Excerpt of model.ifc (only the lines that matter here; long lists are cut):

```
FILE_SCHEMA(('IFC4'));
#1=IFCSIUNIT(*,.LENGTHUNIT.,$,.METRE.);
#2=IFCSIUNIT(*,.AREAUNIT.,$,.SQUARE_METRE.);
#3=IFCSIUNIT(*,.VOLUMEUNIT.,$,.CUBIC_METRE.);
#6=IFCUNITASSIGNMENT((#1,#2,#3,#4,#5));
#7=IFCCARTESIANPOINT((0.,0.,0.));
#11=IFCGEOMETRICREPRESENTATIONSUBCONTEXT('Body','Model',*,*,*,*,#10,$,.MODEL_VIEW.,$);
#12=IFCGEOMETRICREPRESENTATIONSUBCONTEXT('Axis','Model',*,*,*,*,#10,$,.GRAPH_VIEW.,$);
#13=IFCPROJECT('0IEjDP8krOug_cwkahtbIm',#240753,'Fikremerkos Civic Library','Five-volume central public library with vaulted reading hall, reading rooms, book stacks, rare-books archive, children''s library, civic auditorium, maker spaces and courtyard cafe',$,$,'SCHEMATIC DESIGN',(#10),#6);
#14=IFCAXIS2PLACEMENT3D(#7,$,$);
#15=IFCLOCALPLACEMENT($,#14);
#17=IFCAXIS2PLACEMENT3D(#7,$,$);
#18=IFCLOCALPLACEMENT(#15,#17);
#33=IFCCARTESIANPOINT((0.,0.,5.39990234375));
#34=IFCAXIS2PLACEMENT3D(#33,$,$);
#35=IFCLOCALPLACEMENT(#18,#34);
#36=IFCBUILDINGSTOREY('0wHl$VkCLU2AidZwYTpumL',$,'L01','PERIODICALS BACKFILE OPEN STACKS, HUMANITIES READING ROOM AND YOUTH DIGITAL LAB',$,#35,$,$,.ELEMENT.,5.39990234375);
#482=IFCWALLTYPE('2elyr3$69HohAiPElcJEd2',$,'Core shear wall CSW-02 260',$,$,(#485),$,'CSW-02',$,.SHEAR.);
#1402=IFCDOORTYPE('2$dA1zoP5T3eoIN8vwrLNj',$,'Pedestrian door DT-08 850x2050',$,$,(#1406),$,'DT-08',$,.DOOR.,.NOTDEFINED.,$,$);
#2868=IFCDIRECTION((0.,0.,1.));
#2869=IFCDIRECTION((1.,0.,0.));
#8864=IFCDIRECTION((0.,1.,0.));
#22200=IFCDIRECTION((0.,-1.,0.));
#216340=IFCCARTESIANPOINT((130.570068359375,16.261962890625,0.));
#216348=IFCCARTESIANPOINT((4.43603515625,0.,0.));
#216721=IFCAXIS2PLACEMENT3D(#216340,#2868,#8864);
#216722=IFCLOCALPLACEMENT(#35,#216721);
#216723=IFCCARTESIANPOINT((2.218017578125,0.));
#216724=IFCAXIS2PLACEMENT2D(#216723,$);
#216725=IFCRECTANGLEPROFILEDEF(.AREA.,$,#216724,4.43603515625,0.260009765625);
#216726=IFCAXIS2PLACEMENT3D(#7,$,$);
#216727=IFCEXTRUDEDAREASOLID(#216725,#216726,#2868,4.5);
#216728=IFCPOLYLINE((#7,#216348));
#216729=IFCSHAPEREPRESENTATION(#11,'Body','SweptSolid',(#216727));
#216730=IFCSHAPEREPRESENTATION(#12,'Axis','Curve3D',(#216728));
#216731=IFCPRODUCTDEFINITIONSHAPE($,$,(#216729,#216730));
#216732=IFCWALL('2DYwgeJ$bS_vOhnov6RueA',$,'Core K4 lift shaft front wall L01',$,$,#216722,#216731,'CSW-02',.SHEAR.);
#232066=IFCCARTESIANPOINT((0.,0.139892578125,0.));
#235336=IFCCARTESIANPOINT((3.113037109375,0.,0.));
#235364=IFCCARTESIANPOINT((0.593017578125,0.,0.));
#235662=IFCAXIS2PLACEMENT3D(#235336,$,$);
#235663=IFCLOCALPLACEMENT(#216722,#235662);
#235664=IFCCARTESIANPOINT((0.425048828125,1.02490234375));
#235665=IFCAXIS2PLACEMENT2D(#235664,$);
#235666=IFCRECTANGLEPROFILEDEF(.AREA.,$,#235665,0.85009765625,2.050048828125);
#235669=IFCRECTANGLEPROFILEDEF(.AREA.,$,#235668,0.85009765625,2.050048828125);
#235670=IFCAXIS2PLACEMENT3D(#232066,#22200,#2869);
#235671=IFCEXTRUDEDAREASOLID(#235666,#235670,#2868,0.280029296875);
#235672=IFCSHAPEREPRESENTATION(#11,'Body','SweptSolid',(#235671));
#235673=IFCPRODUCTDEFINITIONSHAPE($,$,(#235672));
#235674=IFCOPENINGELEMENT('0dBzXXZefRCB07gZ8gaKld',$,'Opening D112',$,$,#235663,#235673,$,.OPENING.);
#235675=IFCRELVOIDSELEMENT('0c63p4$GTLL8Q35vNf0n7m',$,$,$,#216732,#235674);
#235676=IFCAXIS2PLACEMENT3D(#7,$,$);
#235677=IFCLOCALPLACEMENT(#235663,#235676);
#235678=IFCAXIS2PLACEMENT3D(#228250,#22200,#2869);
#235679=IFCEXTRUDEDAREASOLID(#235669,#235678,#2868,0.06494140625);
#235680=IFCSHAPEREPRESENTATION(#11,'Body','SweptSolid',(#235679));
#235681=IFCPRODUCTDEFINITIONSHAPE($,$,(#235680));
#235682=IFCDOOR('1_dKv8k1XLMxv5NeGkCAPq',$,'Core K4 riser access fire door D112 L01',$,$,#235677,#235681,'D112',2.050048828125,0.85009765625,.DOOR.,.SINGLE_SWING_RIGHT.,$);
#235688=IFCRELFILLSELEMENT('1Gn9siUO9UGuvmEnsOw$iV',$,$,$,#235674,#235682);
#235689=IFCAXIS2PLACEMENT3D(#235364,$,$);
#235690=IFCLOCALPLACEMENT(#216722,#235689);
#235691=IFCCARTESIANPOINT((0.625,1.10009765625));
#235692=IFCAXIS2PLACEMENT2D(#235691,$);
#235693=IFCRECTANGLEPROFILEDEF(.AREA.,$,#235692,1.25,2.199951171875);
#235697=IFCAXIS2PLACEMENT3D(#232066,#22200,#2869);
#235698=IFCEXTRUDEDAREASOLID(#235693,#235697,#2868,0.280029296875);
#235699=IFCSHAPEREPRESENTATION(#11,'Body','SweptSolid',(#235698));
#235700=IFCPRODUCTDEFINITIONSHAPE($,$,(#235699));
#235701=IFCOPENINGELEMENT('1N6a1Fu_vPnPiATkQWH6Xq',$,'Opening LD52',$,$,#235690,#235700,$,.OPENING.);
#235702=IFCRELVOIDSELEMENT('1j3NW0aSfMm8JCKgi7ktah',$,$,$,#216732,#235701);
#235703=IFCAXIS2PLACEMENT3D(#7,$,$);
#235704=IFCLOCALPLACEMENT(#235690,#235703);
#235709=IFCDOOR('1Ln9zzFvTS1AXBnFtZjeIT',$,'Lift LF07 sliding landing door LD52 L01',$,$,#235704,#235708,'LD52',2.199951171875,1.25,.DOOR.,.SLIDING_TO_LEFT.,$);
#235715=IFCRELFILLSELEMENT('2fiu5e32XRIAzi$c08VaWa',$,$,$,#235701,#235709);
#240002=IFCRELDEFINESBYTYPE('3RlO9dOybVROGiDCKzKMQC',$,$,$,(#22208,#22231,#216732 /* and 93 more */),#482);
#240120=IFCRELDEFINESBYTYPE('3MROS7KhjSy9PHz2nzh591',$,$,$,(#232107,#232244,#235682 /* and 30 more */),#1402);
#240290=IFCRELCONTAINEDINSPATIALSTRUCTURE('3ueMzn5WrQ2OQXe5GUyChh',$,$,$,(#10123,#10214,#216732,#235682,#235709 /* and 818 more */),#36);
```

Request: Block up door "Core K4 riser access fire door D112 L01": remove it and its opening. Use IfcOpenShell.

```python
import ifcopenshell
import ifcopenshell.api.feature
import ifcopenshell.api.root
import ifcopenshell.geom
import ifcopenshell.util.shape

model = ifcopenshell.open("model.ifc")
settings = ifcopenshell.geom.settings()


def volume(element):
    """Net volume in cubic metres, openings subtracted."""
    shape = ifcopenshell.geom.create_shape(settings, element)
    return ifcopenshell.util.shape.get_volume(shape.geometry)


door = model.by_guid("1_dKv8k1XLMxv5NeGkCAPq")
opening = door.FillsVoids[0].RelatingOpeningElement
wall = opening.VoidsElements[0].RelatingBuildingElement
before = volume(wall)

ifcopenshell.api.root.remove_product(model, product=door)
ifcopenshell.api.feature.remove_feature(model, feature=opening)

after = volume(wall)

print(f"wall volume {before:.3f} -> {after:.3f} m3")

model.write("model_updated.ifc")
```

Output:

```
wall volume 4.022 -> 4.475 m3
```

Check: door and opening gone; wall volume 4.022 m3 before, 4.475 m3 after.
